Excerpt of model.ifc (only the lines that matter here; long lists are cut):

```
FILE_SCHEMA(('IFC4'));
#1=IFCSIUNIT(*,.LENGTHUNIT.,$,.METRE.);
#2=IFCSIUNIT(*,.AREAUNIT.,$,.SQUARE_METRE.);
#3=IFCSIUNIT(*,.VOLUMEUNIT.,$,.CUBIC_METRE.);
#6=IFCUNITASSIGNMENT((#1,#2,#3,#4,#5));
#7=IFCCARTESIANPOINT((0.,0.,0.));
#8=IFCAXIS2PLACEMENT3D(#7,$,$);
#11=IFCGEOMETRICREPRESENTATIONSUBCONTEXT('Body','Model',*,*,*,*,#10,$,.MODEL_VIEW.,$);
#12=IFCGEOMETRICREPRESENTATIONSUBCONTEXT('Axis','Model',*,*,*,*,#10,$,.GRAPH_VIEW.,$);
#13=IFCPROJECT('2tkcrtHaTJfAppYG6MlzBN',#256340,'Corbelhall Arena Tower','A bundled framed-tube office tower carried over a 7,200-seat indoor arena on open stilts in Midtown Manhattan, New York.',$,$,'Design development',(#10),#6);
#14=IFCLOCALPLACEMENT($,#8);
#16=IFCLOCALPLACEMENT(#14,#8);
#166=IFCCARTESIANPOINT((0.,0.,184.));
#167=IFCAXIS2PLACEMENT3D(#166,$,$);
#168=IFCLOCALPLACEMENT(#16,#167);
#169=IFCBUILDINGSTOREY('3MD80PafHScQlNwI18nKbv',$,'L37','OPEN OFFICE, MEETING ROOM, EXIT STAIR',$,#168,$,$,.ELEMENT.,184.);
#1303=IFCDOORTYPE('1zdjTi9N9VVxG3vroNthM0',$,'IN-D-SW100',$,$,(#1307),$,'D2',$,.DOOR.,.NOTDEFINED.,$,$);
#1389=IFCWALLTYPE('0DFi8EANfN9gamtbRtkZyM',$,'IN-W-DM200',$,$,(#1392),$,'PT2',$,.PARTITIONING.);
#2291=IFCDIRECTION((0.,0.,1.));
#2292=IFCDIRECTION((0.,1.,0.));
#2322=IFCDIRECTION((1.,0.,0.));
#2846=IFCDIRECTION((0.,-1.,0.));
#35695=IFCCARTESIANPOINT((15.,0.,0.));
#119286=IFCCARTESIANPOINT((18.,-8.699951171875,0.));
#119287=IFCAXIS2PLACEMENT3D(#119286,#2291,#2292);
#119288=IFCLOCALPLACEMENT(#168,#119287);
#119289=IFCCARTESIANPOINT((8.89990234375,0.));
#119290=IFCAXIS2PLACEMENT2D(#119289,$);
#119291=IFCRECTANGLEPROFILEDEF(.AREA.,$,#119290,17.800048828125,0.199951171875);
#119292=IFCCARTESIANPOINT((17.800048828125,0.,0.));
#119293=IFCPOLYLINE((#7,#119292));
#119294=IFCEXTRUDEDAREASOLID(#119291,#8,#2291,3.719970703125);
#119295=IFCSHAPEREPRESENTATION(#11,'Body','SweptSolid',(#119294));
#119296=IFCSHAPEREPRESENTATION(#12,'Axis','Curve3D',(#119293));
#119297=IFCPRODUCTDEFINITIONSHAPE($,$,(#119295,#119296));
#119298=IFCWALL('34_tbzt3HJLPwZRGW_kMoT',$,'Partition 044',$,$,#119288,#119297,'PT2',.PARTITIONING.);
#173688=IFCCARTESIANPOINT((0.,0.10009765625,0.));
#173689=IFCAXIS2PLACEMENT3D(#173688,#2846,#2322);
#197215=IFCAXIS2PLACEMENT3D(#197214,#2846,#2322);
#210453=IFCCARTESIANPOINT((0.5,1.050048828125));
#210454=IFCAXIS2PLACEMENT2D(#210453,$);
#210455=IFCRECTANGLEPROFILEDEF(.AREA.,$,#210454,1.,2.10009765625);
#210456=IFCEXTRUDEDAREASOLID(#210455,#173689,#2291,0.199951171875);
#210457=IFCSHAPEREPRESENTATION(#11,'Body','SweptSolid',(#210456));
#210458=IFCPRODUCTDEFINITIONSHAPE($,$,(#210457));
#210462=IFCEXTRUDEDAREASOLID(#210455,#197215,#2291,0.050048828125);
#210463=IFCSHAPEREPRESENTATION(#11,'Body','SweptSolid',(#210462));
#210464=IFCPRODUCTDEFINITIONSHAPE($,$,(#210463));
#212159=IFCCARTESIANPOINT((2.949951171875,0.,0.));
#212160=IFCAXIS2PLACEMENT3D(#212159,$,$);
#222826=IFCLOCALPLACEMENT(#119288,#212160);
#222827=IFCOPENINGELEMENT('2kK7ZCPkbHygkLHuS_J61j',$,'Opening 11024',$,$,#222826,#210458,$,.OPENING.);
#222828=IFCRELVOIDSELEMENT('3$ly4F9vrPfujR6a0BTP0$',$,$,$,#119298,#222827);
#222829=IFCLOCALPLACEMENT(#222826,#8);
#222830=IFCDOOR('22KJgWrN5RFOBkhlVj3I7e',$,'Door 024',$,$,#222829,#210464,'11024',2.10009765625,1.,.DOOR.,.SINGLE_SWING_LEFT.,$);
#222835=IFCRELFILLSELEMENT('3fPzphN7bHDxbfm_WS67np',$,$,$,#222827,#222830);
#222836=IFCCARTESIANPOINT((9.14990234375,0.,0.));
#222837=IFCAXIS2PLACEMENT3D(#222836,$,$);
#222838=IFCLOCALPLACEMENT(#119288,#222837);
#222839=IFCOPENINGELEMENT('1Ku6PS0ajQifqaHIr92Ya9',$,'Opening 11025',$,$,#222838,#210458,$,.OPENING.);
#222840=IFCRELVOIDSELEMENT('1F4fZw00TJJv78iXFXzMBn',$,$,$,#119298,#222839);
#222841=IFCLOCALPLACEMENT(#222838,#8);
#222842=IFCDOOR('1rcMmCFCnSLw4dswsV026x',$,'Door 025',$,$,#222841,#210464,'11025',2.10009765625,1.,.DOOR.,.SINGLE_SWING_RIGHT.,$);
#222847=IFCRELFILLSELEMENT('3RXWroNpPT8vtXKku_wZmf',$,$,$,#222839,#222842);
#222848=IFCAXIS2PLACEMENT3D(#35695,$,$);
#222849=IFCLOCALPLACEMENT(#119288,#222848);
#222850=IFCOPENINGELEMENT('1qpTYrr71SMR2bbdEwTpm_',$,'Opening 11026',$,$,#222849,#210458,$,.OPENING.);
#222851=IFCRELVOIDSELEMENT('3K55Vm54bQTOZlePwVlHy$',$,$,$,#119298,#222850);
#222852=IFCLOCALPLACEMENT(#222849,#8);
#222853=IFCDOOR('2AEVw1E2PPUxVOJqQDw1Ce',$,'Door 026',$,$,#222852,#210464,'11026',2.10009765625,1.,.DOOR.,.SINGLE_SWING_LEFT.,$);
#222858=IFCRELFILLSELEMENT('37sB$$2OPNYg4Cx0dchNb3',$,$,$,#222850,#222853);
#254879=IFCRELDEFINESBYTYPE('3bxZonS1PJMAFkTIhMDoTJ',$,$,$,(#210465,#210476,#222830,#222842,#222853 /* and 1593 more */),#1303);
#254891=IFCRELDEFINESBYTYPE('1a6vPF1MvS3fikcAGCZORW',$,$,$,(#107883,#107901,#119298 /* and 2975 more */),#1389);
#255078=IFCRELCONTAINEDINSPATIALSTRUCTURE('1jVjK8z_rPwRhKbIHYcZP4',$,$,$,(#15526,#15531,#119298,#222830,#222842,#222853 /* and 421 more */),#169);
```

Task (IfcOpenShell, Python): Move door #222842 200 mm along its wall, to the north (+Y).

```python
import ifcopenshell
import ifcopenshell.api.geometry
import ifcopenshell.util.placement
import ifcopenshell.util.unit

model = ifcopenshell.open("model.ifc")
unit_scale = ifcopenshell.util.unit.calculate_unit_scale(model)

door = model.by_guid("1rcMmCFCnSLw4dswsV026x")
opening = door.FillsVoids[0].RelatingOpeningElement
wall = opening.VoidsElements[0].RelatingBuildingElement

wall_matrix = ifcopenshell.util.placement.get_local_placement(wall.ObjectPlacement)
shift = wall_matrix[:3, 0] * 0.2 / unit_scale
before = ifcopenshell.util.placement.get_local_placement(door.ObjectPlacement)[:3, 3].copy()

# The door is placed relative to its opening, so it follows when the opening moves.
matrix = ifcopenshell.util.placement.get_local_placement(opening.ObjectPlacement)
matrix[:3, 3] += shift
ifcopenshell.api.geometry.edit_object_placement(
    model, product=opening, matrix=matrix, is_si=False, should_transform_children=True
)

after = ifcopenshell.util.placement.get_local_placement(door.ObjectPlacement)[:3, 3]
print("door moved by", (after - before).round(3) + 0.0)

model.write("model_edited.ifc")
```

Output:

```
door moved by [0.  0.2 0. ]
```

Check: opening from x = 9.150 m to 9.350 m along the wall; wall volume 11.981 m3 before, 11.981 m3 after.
